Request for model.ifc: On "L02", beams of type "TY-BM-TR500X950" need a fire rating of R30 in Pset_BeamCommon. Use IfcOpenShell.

First a look at what the model holds.

```python
import ifcopenshell
import ifcopenshell.util.element

model = ifcopenshell.open("model.ifc")
print(model.schema)
storey = next(s for s in model.by_type("IfcBuildingStorey") if s.Name == "L02")
beams = [e for e in ifcopenshell.util.element.get_decomposition(storey) if e.is_a("IfcBeam")]
seen = {}
for e in beams:
    element_type = ifcopenshell.util.element.get_type(e)
    key = (element_type.Name if element_type != e and element_type else None, ifcopenshell.util.element.get_pset(e, "Pset_BeamCommon", "FireRating"))
    seen[key] = seen.get(key, 0) + 1
for (name, value), count in sorted(seen.items(), key=str):
    print(count, "x", name, "|", value)
```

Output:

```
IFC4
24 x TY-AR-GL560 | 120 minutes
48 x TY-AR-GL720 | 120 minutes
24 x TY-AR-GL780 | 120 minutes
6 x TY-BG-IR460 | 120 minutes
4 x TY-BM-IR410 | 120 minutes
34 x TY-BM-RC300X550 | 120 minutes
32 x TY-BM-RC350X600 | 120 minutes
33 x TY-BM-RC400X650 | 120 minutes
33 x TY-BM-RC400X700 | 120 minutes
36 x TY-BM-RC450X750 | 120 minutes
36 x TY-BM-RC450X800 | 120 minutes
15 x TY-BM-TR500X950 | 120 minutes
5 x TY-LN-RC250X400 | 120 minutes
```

```python
import ifcopenshell
import ifcopenshell.api.pset
import ifcopenshell.util.element

model = ifcopenshell.open("model.ifc")

storey = next(s for s in model.by_type("IfcBuildingStorey") if s.Name == "L02")
beams = [e for e in ifcopenshell.util.element.get_decomposition(storey) if e.is_a("IfcBeam")]

count = 0
for e in beams:
    element_type = ifcopenshell.util.element.get_type(e)
    if element_type in (None, e) or element_type.Name != "TY-BM-TR500X950":
        continue
    # add_pset returns the element's existing set when there is one.
    pset = ifcopenshell.api.pset.add_pset(model, product=e, name="Pset_BeamCommon")
    ifcopenshell.api.pset.edit_pset(model, pset=pset, properties={"FireRating": "R30"})
    count += 1

print(count, "beams updated")

model.write("model-out.ifc")
```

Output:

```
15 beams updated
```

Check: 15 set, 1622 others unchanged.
